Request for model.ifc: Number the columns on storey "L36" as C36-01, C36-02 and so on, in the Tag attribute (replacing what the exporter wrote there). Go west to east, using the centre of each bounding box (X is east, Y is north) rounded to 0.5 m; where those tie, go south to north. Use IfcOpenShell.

First a look at what the model holds.

```python
import ifcopenshell
import ifcopenshell.util.element
import ifcopenshell.util.placement

model = ifcopenshell.open("model.ifc")
print(model.schema)
storey = next(s for s in model.by_type("IfcBuildingStorey") if s.Name == "L36")
columns = [e for e in ifcopenshell.util.element.get_decomposition(storey) if e.is_a("IfcColumn")]
for e in sorted(columns, key=lambda e: e.id()):
    origin = ifcopenshell.util.placement.get_local_placement(e.ObjectPlacement)[:3, 3]
    print(e.id(), e.Tag, e.Name, origin.round(2) + 0.0, sep=" | ")
```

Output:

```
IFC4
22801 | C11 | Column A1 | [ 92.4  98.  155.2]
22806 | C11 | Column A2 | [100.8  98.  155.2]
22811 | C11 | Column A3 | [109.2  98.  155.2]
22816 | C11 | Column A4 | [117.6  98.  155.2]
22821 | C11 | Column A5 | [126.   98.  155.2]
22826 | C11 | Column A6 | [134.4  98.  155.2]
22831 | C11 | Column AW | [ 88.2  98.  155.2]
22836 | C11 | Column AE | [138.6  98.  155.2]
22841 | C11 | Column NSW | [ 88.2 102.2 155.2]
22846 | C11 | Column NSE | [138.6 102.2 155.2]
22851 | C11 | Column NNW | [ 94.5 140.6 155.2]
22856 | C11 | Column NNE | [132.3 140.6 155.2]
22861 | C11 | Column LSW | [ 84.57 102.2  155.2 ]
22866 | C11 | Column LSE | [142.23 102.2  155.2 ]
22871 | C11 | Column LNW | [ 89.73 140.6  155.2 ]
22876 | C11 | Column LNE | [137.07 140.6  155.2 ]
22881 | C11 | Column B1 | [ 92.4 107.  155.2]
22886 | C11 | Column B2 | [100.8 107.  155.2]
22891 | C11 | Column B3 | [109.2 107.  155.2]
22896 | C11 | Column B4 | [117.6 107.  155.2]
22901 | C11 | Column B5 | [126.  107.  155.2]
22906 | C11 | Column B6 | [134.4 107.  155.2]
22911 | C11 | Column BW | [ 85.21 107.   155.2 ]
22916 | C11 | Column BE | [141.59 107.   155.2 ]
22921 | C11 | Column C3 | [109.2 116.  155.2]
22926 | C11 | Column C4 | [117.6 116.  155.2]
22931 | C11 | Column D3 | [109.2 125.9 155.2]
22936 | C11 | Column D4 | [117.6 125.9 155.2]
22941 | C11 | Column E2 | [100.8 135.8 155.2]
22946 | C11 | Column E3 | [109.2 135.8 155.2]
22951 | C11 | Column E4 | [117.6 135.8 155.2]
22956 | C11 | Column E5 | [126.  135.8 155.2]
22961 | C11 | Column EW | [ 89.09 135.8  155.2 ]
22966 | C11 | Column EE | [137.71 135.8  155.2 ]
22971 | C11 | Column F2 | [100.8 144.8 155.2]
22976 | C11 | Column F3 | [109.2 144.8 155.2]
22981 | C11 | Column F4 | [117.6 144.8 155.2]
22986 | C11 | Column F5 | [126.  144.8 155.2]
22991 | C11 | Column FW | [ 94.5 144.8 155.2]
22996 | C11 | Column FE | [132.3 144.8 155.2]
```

```python
import ifcopenshell
import ifcopenshell.geom
import ifcopenshell.util.element
import ifcopenshell.util.shape

model = ifcopenshell.open("model.ifc")
settings = ifcopenshell.geom.settings()
settings.set("use-world-coords", True)


def centre(element):
    shape = ifcopenshell.geom.create_shape(settings, element)
    return ifcopenshell.util.shape.get_bbox_centroid(shape.geometry)


storey = next(s for s in model.by_type("IfcBuildingStorey") if s.Name == "L36")
columns = [e for e in ifcopenshell.util.element.get_decomposition(storey) if e.is_a("IfcColumn")]

# Insertion points can sit at a corner or the storey origin, so sort by the geometry (in metres).
centres = {e: centre(e) for e in columns}
columns.sort(key=lambda e: (round(centres[e][0] / 0.5), centres[e][1]))

for i, e in enumerate(columns, start=1):
    number = f"C36-{i:02d}"
    e.Tag = number
    print(e.id(), number)

model.write("model_edited.ifc")
```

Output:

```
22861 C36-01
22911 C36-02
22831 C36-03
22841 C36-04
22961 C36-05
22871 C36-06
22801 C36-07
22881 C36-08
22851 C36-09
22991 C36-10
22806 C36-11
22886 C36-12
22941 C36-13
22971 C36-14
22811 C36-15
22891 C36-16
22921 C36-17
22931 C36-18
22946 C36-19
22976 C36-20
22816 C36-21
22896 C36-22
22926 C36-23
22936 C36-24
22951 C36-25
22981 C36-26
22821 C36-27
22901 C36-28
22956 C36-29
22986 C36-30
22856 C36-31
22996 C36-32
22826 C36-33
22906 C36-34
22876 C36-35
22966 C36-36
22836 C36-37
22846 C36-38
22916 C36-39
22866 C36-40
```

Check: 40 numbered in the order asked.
